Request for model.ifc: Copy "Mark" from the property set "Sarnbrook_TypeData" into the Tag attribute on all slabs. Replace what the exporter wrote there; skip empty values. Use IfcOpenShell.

First a look at what the model holds.

```python
import ifcopenshell
import ifcopenshell.util.element

model = ifcopenshell.open("model.ifc")
print(model.schema)
slabs = model.by_type("IfcSlab")
print(len(slabs), "slabs")
for e in slabs[:8]:
    source = ifcopenshell.util.element.get_pset(e, "Sarnbrook_TypeData", "Mark")
    target = e.Tag
    print(e.id(), repr(source), repr(target), sep=" | ")
```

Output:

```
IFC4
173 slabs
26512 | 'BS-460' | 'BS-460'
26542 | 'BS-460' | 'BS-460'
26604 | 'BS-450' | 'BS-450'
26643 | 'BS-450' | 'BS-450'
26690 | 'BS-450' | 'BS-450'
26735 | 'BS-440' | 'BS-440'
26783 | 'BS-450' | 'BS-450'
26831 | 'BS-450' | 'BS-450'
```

```python
import ifcopenshell
import ifcopenshell.util.element

model = ifcopenshell.open("model.ifc")

count = 0
for e in model.by_type("IfcSlab"):
    value = ifcopenshell.util.element.get_pset(e, "Sarnbrook_TypeData", "Mark")
    current = e.Tag
    if not value or not value.strip() or current == value:
        continue
    e.Tag = value
    count += 1

print(count, "slabs updated")

model.write("model_rev.ifc")
```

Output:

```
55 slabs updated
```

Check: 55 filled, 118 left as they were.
